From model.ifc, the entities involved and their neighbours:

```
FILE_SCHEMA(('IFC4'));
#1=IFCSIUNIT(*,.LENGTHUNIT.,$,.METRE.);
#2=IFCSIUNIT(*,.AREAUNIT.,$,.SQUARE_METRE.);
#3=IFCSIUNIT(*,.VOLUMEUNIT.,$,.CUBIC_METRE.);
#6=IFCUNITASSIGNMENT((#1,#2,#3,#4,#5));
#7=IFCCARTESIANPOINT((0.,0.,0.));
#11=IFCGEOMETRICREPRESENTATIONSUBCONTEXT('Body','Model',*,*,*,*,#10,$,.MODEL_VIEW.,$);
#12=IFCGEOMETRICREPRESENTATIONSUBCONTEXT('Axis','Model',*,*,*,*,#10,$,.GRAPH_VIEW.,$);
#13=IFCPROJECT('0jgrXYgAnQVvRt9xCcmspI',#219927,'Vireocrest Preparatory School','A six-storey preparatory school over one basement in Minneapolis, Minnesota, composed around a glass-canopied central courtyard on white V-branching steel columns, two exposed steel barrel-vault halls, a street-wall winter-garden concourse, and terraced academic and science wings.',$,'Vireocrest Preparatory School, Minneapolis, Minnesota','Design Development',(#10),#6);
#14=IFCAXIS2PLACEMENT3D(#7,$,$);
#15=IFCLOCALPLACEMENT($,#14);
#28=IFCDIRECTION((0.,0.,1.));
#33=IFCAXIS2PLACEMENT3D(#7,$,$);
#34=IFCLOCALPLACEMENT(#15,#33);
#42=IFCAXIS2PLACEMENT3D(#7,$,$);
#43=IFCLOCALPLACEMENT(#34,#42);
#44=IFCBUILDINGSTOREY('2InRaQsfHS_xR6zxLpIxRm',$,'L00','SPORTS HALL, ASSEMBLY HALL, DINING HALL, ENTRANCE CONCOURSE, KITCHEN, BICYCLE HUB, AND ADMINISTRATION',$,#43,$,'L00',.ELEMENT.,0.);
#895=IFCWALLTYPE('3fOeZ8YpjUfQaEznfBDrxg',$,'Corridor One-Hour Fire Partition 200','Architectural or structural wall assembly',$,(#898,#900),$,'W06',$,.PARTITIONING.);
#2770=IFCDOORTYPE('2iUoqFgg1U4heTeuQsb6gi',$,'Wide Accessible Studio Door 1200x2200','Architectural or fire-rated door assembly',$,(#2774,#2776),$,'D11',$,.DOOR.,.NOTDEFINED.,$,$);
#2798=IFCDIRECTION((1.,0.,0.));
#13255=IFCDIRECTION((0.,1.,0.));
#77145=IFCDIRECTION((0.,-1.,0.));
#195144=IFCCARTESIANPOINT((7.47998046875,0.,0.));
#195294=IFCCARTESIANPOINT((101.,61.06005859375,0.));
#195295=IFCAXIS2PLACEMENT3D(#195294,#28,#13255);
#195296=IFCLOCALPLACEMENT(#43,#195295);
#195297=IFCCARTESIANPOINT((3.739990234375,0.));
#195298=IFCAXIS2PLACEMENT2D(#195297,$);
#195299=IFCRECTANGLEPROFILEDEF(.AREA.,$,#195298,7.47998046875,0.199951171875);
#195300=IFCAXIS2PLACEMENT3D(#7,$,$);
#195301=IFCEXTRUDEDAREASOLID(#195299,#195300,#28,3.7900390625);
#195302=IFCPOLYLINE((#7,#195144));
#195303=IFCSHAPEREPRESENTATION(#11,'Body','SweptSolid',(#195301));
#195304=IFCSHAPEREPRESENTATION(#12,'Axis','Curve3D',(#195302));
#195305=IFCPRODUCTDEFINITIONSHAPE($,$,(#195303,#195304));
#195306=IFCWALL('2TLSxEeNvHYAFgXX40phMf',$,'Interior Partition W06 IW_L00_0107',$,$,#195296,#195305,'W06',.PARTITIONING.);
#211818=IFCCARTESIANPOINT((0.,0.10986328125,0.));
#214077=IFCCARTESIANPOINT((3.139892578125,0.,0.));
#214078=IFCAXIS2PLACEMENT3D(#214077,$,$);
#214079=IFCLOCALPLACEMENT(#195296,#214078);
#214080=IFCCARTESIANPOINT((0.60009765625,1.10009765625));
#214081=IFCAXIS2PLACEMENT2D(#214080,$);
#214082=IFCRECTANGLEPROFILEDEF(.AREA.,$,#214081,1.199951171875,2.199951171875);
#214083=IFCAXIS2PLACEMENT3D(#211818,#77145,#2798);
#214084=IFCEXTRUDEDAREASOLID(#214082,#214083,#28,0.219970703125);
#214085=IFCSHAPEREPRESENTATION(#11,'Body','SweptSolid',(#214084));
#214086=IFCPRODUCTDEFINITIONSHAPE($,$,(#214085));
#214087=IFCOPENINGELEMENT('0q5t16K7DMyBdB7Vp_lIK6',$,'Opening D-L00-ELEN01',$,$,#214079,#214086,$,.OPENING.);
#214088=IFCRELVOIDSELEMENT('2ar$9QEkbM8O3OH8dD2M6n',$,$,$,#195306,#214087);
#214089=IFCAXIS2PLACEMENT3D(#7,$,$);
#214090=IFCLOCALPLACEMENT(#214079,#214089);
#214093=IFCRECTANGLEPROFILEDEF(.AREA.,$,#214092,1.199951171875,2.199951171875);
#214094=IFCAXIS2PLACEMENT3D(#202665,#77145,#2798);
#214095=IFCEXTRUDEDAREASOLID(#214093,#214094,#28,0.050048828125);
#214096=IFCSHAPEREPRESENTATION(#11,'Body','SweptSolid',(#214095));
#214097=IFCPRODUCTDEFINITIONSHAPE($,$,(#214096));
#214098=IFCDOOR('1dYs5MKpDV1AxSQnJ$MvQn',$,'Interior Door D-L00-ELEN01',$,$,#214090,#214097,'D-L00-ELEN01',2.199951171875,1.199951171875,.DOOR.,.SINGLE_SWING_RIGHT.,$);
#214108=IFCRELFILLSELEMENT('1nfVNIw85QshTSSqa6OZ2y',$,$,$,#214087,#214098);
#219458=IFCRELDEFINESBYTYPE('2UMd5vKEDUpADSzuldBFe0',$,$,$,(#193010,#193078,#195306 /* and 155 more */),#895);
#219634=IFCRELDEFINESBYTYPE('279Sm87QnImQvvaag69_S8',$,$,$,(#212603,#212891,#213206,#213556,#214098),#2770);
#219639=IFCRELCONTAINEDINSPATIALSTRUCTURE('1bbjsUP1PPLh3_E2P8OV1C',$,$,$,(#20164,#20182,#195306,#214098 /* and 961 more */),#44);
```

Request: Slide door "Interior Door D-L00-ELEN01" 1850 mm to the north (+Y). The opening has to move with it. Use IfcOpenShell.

```python
import ifcopenshell
import ifcopenshell.api.geometry
import ifcopenshell.util.placement
import ifcopenshell.util.unit

model = ifcopenshell.open("model.ifc")
unit_scale = ifcopenshell.util.unit.calculate_unit_scale(model)

door = model.by_id(214098)
opening = door.FillsVoids[0].RelatingOpeningElement
wall = opening.VoidsElements[0].RelatingBuildingElement

wall_matrix = ifcopenshell.util.placement.get_local_placement(wall.ObjectPlacement)
shift = wall_matrix[:3, 0] * 1.85 / unit_scale
before = ifcopenshell.util.placement.get_local_placement(door.ObjectPlacement)[:3, 3].copy()

# The door is placed relative to its opening, so it follows when the opening moves.
matrix = ifcopenshell.util.placement.get_local_placement(opening.ObjectPlacement)
matrix[:3, 3] += shift
ifcopenshell.api.geometry.edit_object_placement(
    model, product=opening, matrix=matrix, is_si=False, should_transform_children=True
)

after = ifcopenshell.util.placement.get_local_placement(door.ObjectPlacement)[:3, 3]
print("door moved by", (after - before).round(3) + 0.0)

model.write("model_updated.ifc")
```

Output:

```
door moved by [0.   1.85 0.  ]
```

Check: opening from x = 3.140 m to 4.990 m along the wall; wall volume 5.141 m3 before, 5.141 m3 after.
